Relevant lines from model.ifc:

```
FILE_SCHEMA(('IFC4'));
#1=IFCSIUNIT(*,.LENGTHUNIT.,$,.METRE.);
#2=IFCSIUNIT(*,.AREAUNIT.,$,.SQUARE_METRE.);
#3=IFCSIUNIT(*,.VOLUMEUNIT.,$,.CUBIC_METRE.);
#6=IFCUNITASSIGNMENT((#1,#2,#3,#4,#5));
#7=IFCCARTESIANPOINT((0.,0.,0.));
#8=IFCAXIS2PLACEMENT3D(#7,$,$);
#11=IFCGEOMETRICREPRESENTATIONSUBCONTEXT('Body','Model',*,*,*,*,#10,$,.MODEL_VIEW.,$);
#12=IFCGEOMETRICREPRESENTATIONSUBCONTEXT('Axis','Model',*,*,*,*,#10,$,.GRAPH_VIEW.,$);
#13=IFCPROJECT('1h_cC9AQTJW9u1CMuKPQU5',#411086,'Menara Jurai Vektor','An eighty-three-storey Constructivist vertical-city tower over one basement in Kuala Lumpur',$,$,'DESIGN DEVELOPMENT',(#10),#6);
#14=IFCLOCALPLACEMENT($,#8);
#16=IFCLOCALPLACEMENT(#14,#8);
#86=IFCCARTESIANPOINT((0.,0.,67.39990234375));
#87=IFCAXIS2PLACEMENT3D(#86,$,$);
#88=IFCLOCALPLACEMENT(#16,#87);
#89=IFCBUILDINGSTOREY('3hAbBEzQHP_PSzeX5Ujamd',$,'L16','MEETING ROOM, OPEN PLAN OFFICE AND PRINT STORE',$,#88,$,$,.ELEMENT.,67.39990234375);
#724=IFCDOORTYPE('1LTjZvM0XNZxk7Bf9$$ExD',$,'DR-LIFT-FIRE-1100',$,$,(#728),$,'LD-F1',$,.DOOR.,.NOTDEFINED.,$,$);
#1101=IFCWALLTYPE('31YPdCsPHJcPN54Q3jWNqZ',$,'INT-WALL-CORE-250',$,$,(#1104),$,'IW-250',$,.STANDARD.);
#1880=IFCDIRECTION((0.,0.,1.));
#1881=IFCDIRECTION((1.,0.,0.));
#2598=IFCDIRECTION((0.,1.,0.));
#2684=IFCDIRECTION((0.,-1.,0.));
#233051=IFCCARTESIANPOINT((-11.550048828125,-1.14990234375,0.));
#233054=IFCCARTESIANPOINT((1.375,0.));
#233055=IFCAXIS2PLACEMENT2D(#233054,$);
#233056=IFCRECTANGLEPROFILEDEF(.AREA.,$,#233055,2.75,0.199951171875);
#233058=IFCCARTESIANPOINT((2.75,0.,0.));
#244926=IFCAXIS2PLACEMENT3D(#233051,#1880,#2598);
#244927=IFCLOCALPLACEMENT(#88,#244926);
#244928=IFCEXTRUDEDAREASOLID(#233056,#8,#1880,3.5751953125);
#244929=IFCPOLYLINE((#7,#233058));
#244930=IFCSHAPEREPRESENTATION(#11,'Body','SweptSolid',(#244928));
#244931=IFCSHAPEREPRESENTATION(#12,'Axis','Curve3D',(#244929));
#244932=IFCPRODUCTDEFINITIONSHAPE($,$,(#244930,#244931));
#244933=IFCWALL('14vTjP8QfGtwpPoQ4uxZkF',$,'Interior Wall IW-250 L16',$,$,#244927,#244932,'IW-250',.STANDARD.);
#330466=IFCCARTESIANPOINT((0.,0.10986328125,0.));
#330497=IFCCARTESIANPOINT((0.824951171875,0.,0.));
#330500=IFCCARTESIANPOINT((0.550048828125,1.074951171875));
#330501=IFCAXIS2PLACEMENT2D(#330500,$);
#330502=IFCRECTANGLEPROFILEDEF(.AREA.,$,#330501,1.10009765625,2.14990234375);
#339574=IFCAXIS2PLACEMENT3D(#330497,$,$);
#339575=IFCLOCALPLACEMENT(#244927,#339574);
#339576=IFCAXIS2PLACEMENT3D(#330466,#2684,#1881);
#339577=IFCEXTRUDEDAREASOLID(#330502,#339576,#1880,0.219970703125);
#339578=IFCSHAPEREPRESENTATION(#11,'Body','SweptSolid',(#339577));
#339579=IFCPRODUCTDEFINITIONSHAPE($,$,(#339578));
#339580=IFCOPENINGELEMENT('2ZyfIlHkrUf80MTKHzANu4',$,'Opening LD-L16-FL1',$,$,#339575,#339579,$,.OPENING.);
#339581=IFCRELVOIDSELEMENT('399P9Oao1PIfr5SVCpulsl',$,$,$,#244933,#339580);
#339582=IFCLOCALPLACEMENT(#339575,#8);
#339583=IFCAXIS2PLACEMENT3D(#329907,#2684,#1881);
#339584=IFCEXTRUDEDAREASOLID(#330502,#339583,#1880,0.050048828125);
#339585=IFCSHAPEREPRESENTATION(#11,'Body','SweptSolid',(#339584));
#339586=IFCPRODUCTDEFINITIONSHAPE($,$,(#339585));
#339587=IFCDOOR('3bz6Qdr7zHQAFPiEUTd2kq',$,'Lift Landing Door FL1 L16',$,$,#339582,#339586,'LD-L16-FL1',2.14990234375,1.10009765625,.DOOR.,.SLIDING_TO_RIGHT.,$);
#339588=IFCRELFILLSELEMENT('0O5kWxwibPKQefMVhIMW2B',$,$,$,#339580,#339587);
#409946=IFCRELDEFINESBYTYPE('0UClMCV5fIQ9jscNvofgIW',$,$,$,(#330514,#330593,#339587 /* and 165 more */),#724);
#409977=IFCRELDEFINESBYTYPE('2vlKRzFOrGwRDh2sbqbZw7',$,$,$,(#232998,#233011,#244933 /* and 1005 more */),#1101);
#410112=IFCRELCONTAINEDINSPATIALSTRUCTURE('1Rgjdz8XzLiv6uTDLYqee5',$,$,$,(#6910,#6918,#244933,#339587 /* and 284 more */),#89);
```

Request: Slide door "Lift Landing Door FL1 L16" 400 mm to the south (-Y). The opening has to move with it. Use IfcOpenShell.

```python
import ifcopenshell
import ifcopenshell.api.geometry
import ifcopenshell.util.placement
import ifcopenshell.util.unit

model = ifcopenshell.open("model.ifc")
unit_scale = ifcopenshell.util.unit.calculate_unit_scale(model)

door = model.by_guid("3bz6Qdr7zHQAFPiEUTd2kq")
opening = door.FillsVoids[0].RelatingOpeningElement
wall = opening.VoidsElements[0].RelatingBuildingElement

wall_matrix = ifcopenshell.util.placement.get_local_placement(wall.ObjectPlacement)
shift = wall_matrix[:3, 0] * -0.4 / unit_scale
before = ifcopenshell.util.placement.get_local_placement(door.ObjectPlacement)[:3, 3].copy()

# The door is placed relative to its opening, so it follows when the opening moves.
matrix = ifcopenshell.util.placement.get_local_placement(opening.ObjectPlacement)
matrix[:3, 3] += shift
ifcopenshell.api.geometry.edit_object_placement(
    model, product=opening, matrix=matrix, is_si=False, should_transform_children=True
)

after = ifcopenshell.util.placement.get_local_placement(door.ObjectPlacement)[:3, 3]
print("door moved by", (after - before).round(3) + 0.0)

model.write("model_updated.ifc")
```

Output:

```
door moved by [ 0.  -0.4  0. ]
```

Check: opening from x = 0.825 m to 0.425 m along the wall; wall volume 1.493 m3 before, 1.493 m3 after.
